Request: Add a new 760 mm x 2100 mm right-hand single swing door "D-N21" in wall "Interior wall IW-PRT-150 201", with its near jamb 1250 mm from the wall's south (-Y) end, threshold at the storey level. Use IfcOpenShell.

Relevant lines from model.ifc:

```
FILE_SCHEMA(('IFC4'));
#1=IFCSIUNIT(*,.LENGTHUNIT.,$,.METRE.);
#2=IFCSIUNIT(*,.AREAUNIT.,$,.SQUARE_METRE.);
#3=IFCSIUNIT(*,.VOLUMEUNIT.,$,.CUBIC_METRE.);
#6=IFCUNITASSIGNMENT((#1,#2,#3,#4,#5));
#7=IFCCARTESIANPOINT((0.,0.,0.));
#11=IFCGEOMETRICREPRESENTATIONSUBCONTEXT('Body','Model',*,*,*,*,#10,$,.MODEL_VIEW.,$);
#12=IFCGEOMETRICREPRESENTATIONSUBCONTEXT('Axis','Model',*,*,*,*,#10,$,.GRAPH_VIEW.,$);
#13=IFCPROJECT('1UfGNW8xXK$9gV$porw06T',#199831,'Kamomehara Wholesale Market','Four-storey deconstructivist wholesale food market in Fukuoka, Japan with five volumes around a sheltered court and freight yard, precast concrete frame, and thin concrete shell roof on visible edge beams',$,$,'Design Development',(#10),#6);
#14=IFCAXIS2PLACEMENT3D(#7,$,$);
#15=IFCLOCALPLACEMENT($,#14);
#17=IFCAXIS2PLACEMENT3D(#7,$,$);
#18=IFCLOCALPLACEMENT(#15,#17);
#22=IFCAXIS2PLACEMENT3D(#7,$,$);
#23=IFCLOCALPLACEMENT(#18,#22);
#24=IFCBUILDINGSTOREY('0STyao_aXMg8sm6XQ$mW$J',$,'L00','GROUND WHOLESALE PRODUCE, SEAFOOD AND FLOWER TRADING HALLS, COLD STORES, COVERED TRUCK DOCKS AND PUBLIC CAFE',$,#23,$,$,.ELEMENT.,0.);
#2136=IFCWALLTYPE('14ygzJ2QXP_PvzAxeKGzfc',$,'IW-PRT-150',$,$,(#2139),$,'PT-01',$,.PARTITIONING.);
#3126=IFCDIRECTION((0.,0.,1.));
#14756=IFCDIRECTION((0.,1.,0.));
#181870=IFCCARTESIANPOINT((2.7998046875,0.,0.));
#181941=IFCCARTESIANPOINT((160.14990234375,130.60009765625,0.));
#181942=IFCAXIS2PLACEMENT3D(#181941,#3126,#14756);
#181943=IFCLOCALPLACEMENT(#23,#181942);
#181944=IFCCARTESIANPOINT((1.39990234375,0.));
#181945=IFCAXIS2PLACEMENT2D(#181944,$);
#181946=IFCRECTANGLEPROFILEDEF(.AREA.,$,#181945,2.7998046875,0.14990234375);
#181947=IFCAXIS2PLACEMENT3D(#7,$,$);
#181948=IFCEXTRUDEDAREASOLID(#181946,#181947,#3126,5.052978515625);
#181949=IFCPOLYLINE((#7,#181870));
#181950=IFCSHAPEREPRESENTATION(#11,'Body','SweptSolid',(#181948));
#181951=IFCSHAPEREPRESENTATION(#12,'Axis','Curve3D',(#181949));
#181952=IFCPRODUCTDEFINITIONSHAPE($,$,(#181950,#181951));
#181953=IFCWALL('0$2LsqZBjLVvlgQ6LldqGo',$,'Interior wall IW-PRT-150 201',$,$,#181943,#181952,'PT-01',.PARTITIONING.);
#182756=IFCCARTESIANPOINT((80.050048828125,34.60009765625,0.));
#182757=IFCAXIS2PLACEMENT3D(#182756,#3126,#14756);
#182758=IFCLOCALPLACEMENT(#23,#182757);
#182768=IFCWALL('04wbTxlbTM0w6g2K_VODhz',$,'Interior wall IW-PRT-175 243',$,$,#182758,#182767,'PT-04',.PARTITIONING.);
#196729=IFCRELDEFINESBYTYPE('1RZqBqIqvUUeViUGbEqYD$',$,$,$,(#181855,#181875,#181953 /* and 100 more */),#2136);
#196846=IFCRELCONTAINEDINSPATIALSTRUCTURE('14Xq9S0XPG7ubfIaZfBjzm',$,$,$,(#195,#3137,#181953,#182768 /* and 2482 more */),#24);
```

```python
import numpy as np
import ifcopenshell
import ifcopenshell.api.feature
import ifcopenshell.api.geometry
import ifcopenshell.api.root
import ifcopenshell.api.spatial
import ifcopenshell.geom
import ifcopenshell.util.element
import ifcopenshell.util.placement
import ifcopenshell.util.representation
import ifcopenshell.util.shape
import ifcopenshell.util.unit

model = ifcopenshell.open("model.ifc")
unit_scale = ifcopenshell.util.unit.calculate_unit_scale(model)
settings = ifcopenshell.geom.settings()


def volume(element):
    """Net volume in cubic metres, openings subtracted."""
    shape = ifcopenshell.geom.create_shape(settings, element)
    return ifcopenshell.util.shape.get_volume(shape.geometry)


wall = model.by_guid("0$2LsqZBjLVvlgQ6LldqGo")
storey = ifcopenshell.util.element.get_container(wall, ifc_class="IfcBuildingStorey")
context = ifcopenshell.util.representation.get_context(model, "Model", "Body", "MODEL_VIEW")
before = volume(wall)

width, height, from_end, sill = 0.76, 2.1, 1.25, 0.0  # metres

# The wall runs along its own X axis, and the end named is its -X end.
wall_shape = ifcopenshell.geom.create_shape(settings, wall)
x, y, z = ifcopenshell.util.shape.get_vertices(wall_shape.geometry).T
start = x.min() + from_end
face, thickness = float(y.min()), float(y.max() - y.min())
wall_matrix = ifcopenshell.util.placement.get_local_placement(wall.ObjectPlacement)
level = ifcopenshell.util.placement.get_local_placement(storey.ObjectPlacement)[2, 3]


def in_wall(x, y):
    """Placement at x, y metres in the wall's axes, at sill height."""
    matrix = wall_matrix.copy()
    matrix[:, 3] = wall_matrix @ np.array([x / unit_scale, y / unit_scale, 0.0, 1.0])
    matrix[2, 3] = level + sill / unit_scale
    return matrix


# Opening: a box that overshoots both wall faces by 50 mm.
opening = ifcopenshell.api.root.create_entity(model, ifc_class="IfcOpeningElement", predefined_type="OPENING")
box = ifcopenshell.api.geometry.add_wall_representation(
    model, context=context, length=width, height=height, thickness=thickness + 0.1
)
ifcopenshell.api.geometry.assign_representation(model, product=opening, representation=box)
ifcopenshell.api.geometry.edit_object_placement(model, product=opening, matrix=in_wall(start, face - 0.05), is_si=False)
ifcopenshell.api.feature.add_feature(model, feature=opening, element=wall)

door = ifcopenshell.api.root.create_entity(model, ifc_class="IfcDoor", name="D-N21", predefined_type="DOOR")
door.OverallWidth, door.OverallHeight = width / unit_scale, height / unit_scale
door.OperationType = "SINGLE_SWING_RIGHT"
body = ifcopenshell.api.geometry.add_door_representation(
    model,
    context=context,
    overall_width=door.OverallWidth,
    overall_height=door.OverallHeight,
    operation_type="SINGLE_SWING_RIGHT",
    lining_properties={"LiningDepth": thickness / unit_scale, "ThresholdDepth": thickness / unit_scale},
)
ifcopenshell.api.geometry.assign_representation(model, product=door, representation=body)
ifcopenshell.api.spatial.assign_container(model, products=[door], relating_structure=storey)
ifcopenshell.api.feature.add_filling(model, opening=opening, element=door)

# The lining spans the wall, so the door starts at the wall face.
ifcopenshell.api.geometry.edit_object_placement(model, product=door, matrix=in_wall(start, face), is_si=False)

after = volume(wall)

print(f"wall volume {before:.3f} -> {after:.3f} m3")

model.write("model_edited.ifc")
```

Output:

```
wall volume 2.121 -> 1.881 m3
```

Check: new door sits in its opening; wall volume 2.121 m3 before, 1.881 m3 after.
